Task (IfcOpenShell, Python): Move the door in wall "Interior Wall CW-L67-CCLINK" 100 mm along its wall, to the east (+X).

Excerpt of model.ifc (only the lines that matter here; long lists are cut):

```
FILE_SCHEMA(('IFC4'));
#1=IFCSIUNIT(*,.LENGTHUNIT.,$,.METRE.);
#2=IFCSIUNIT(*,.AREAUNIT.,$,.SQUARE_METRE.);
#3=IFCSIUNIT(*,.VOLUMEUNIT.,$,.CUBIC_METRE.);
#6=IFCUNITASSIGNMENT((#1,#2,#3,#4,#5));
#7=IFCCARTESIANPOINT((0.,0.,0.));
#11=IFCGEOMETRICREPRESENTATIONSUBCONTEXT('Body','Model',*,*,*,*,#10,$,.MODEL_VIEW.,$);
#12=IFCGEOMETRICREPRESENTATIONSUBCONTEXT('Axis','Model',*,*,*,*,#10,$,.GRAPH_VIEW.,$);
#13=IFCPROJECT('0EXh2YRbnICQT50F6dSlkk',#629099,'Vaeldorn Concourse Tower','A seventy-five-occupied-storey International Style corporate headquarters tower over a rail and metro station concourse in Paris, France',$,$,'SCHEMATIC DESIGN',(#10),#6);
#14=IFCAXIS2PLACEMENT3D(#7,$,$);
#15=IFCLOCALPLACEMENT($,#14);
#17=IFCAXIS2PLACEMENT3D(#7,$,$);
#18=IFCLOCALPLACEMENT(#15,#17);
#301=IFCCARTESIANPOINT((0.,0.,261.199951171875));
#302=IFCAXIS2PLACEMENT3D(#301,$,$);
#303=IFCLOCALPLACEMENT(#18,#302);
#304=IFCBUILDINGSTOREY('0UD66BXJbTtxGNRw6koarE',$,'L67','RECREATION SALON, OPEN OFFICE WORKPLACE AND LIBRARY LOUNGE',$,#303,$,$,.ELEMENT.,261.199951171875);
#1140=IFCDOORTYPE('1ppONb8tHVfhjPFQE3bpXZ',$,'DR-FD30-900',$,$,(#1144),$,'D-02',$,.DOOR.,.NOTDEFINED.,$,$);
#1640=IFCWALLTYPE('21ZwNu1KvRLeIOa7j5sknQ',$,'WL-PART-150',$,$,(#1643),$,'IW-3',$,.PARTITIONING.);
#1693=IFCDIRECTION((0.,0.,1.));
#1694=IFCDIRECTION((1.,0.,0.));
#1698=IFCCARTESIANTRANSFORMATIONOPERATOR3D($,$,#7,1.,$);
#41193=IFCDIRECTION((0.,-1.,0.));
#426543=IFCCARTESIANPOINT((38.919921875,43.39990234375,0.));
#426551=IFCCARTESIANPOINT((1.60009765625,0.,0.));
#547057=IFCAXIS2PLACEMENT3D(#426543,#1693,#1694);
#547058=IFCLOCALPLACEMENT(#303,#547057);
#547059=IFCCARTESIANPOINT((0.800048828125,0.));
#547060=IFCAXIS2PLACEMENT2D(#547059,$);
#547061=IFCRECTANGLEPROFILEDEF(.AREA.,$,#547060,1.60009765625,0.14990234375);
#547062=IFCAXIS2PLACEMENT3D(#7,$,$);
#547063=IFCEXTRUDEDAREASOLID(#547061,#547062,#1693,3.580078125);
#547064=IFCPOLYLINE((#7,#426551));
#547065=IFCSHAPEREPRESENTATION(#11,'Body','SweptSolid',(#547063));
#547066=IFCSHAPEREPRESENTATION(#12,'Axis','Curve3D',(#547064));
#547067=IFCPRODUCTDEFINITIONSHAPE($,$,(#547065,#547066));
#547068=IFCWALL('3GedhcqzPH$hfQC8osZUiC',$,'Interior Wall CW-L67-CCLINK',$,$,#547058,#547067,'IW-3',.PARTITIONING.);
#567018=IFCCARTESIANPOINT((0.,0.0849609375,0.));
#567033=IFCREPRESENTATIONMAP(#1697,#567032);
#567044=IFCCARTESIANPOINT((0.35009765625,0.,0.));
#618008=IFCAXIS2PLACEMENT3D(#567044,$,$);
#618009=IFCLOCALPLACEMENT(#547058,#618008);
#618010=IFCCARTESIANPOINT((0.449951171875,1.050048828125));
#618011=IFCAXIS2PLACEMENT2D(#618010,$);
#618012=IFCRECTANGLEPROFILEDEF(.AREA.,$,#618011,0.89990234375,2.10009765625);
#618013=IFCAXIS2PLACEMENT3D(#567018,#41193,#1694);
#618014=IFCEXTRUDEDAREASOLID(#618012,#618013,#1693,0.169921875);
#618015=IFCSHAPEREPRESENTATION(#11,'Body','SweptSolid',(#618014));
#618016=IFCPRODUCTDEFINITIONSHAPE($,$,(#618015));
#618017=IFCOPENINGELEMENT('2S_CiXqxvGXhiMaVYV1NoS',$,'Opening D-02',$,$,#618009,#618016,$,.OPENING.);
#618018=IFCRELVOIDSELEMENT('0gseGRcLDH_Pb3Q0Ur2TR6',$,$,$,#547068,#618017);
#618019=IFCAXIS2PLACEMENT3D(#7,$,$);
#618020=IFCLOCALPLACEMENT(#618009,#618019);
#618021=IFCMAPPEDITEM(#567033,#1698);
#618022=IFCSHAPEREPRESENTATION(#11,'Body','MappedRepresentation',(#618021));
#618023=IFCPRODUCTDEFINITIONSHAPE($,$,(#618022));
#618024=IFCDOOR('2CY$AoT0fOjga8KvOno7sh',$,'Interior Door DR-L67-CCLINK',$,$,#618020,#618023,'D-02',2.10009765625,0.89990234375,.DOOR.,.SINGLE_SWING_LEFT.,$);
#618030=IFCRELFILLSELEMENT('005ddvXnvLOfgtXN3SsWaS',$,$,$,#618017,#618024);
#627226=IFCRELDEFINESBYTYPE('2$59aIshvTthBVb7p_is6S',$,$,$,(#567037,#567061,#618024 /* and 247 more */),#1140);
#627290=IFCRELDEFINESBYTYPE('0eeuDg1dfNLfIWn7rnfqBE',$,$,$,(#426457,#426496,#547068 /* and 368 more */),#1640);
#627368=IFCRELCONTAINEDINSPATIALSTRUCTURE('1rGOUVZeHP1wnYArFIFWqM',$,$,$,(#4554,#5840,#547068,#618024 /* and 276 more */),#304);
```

```python
import ifcopenshell
import ifcopenshell.api.geometry
import ifcopenshell.util.placement
import ifcopenshell.util.unit

model = ifcopenshell.open("model.ifc")
unit_scale = ifcopenshell.util.unit.calculate_unit_scale(model)

door = model.by_guid("2CY$AoT0fOjga8KvOno7sh")
opening = door.FillsVoids[0].RelatingOpeningElement
wall = opening.VoidsElements[0].RelatingBuildingElement

wall_matrix = ifcopenshell.util.placement.get_local_placement(wall.ObjectPlacement)
shift = wall_matrix[:3, 0] * 0.1 / unit_scale
before = ifcopenshell.util.placement.get_local_placement(door.ObjectPlacement)[:3, 3].copy()

# The door is placed relative to its opening, so it follows when the opening moves.
matrix = ifcopenshell.util.placement.get_local_placement(opening.ObjectPlacement)
matrix[:3, 3] += shift
ifcopenshell.api.geometry.edit_object_placement(
    model, product=opening, matrix=matrix, is_si=False, should_transform_children=True
)

after = ifcopenshell.util.placement.get_local_placement(door.ObjectPlacement)[:3, 3]
print("door moved by", (after - before).round(3) + 0.0)

model.write("model_rev.ifc")
```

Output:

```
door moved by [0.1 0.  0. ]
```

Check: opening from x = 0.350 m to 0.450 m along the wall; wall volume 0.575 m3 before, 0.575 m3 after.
